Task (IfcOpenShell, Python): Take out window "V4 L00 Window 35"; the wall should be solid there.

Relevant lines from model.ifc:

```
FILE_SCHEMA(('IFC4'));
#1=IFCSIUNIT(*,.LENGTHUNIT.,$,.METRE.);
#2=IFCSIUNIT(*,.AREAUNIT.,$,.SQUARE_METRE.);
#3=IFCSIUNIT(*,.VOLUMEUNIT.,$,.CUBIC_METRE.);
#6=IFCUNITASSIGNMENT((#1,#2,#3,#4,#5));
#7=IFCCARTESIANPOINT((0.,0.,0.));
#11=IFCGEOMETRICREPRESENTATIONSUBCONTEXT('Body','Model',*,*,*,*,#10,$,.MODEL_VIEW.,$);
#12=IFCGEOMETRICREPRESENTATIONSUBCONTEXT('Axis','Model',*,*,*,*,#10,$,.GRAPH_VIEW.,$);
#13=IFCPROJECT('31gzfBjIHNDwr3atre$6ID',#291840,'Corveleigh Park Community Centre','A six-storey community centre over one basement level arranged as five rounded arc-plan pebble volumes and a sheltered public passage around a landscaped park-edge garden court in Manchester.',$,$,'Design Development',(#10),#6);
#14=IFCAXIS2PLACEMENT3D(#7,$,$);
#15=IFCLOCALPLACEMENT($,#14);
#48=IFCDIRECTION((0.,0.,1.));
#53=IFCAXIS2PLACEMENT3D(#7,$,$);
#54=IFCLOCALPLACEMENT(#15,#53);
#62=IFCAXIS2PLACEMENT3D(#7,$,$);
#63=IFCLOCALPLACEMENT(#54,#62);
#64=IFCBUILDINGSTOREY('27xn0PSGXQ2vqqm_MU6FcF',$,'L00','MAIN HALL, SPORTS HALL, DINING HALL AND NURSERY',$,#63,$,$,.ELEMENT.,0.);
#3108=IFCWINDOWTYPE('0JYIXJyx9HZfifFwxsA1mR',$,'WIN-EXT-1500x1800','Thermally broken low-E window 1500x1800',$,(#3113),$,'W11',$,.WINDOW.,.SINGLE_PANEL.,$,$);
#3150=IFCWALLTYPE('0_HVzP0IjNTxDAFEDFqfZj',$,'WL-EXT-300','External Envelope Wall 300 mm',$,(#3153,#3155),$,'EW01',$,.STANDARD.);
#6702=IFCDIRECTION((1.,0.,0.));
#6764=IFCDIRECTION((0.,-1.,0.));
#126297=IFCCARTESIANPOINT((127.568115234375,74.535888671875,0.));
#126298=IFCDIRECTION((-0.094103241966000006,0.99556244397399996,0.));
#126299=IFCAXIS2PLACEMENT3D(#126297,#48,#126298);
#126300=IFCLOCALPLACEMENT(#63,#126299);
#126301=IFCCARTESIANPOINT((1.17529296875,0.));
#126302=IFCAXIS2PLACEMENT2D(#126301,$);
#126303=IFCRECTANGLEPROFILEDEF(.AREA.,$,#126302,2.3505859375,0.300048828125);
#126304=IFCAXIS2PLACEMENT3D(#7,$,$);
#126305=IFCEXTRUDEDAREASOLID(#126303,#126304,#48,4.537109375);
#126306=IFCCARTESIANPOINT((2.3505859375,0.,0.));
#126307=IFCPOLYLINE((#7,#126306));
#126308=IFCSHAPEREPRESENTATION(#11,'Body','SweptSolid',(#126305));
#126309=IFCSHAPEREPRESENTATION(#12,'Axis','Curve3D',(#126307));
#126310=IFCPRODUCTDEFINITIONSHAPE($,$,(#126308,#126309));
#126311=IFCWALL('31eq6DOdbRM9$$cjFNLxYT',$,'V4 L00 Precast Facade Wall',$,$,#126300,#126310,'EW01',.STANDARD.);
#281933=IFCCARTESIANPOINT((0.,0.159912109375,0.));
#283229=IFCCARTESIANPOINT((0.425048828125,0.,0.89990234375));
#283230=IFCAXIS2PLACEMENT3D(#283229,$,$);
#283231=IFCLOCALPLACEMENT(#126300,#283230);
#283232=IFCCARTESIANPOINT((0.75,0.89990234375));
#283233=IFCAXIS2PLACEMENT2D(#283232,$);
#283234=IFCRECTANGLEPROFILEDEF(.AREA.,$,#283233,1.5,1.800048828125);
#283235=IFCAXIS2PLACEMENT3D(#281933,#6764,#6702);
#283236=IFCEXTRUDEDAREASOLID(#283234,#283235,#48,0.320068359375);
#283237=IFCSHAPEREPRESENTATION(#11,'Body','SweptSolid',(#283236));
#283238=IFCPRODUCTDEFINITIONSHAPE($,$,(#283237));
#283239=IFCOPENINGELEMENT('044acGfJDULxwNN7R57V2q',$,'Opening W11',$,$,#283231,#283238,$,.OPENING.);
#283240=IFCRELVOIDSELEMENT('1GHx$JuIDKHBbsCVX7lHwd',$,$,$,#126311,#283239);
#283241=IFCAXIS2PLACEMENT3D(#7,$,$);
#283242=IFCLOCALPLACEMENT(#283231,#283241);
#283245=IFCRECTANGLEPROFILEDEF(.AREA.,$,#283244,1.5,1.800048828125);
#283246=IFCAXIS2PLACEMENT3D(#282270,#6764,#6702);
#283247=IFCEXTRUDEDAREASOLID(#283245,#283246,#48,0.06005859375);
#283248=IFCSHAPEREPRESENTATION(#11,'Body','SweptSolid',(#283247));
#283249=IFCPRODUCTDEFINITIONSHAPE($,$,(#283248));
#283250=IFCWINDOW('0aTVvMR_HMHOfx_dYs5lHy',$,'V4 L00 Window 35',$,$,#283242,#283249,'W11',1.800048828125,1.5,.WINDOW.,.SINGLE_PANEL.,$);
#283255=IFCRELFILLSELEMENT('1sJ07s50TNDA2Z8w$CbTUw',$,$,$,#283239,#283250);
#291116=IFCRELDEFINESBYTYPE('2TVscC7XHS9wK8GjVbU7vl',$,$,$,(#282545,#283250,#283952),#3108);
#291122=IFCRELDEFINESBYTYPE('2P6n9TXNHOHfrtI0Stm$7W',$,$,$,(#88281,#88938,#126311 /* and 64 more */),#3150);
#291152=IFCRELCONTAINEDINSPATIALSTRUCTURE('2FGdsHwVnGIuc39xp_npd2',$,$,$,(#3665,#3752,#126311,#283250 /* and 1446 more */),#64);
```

```python
import ifcopenshell
import ifcopenshell.api.feature
import ifcopenshell.api.root
import ifcopenshell.geom
import ifcopenshell.util.shape

model = ifcopenshell.open("model.ifc")
settings = ifcopenshell.geom.settings()


def volume(element):
    """Net volume in cubic metres, openings subtracted."""
    shape = ifcopenshell.geom.create_shape(settings, element)
    return ifcopenshell.util.shape.get_volume(shape.geometry)


window = model.by_guid("0aTVvMR_HMHOfx_dYs5lHy")
opening = window.FillsVoids[0].RelatingOpeningElement
wall = opening.VoidsElements[0].RelatingBuildingElement
before = volume(wall)

ifcopenshell.api.root.remove_product(model, product=window)
ifcopenshell.api.feature.remove_feature(model, feature=opening)

after = volume(wall)

print(f"wall volume {before:.3f} -> {after:.3f} m3")

model.write("model-out.ifc")
```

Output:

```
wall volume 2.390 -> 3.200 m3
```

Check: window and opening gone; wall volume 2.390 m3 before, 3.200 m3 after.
